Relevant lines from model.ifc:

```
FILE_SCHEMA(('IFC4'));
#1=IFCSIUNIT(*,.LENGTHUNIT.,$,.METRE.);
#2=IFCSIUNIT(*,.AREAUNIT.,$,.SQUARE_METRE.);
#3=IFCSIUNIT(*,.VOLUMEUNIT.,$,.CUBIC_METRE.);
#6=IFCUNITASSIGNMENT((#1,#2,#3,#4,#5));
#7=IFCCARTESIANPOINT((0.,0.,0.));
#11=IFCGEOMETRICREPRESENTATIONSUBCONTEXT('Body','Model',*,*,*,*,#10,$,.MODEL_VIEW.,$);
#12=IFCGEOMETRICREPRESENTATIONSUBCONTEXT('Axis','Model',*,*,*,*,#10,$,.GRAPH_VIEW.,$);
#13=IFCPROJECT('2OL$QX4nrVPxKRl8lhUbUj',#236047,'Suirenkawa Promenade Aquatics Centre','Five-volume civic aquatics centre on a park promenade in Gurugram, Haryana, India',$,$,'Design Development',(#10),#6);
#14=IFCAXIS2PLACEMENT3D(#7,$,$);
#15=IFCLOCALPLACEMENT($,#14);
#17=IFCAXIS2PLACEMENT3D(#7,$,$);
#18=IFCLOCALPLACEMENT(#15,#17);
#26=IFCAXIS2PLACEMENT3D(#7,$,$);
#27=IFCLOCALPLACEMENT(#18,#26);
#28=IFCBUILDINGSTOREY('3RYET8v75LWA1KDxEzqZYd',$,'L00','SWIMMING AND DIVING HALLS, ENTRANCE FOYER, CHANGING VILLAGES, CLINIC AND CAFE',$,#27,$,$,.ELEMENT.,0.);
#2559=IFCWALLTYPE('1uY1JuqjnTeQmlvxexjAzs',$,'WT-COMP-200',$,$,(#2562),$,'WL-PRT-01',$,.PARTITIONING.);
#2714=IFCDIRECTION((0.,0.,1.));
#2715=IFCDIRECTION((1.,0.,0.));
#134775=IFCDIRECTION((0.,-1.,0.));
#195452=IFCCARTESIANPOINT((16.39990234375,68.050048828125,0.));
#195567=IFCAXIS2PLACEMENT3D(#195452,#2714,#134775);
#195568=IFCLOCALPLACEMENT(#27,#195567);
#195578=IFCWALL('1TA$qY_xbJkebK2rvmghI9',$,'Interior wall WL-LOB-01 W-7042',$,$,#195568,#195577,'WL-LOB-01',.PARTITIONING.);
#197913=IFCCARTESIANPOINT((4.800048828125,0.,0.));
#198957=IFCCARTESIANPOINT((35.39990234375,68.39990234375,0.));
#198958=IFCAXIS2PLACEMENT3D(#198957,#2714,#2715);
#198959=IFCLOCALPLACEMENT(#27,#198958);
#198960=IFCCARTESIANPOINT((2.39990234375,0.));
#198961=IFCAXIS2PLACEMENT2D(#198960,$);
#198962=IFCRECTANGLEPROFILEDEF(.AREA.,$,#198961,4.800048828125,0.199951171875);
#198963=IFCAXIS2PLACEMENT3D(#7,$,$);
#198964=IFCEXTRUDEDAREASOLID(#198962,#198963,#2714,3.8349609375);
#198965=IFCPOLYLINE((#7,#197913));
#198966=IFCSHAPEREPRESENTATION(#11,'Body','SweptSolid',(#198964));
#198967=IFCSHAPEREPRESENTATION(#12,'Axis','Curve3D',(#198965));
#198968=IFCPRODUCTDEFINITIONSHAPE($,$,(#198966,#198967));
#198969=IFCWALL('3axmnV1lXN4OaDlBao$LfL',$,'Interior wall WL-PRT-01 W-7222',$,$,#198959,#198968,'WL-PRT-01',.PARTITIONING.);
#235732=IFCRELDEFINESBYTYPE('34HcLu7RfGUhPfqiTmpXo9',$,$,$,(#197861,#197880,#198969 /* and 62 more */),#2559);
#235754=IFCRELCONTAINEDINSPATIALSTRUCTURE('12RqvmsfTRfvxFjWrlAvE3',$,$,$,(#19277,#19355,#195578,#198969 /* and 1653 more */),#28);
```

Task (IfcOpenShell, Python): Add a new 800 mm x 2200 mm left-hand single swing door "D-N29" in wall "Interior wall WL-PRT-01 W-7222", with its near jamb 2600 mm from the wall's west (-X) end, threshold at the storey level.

```python
import numpy as np
import ifcopenshell
import ifcopenshell.api.feature
import ifcopenshell.api.geometry
import ifcopenshell.api.root
import ifcopenshell.api.spatial
import ifcopenshell.geom
import ifcopenshell.util.element
import ifcopenshell.util.placement
import ifcopenshell.util.representation
import ifcopenshell.util.shape
import ifcopenshell.util.unit

model = ifcopenshell.open("model.ifc")
unit_scale = ifcopenshell.util.unit.calculate_unit_scale(model)
settings = ifcopenshell.geom.settings()


def volume(element):
    """Net volume in cubic metres, openings subtracted."""
    shape = ifcopenshell.geom.create_shape(settings, element)
    return ifcopenshell.util.shape.get_volume(shape.geometry)


wall = model.by_guid("3axmnV1lXN4OaDlBao$LfL")
storey = ifcopenshell.util.element.get_container(wall, ifc_class="IfcBuildingStorey")
context = ifcopenshell.util.representation.get_context(model, "Model", "Body", "MODEL_VIEW")
before = volume(wall)

width, height, from_end, sill = 0.8, 2.2, 2.6, 0.0  # metres

# The wall runs along its own X axis, and the end named is its -X end.
wall_shape = ifcopenshell.geom.create_shape(settings, wall)
x, y, z = ifcopenshell.util.shape.get_vertices(wall_shape.geometry).T
start = x.min() + from_end
face, thickness = float(y.min()), float(y.max() - y.min())
wall_matrix = ifcopenshell.util.placement.get_local_placement(wall.ObjectPlacement)
level = ifcopenshell.util.placement.get_local_placement(storey.ObjectPlacement)[2, 3]


def in_wall(x, y):
    """Placement at x, y metres in the wall's axes, at sill height."""
    matrix = wall_matrix.copy()
    matrix[:, 3] = wall_matrix @ np.array([x / unit_scale, y / unit_scale, 0.0, 1.0])
    matrix[2, 3] = level + sill / unit_scale
    return matrix


# Opening: a box that overshoots both wall faces by 50 mm.
opening = ifcopenshell.api.root.create_entity(model, ifc_class="IfcOpeningElement", predefined_type="OPENING")
box = ifcopenshell.api.geometry.add_wall_representation(
    model, context=context, length=width, height=height, thickness=thickness + 0.1
)
ifcopenshell.api.geometry.assign_representation(model, product=opening, representation=box)
ifcopenshell.api.geometry.edit_object_placement(model, product=opening, matrix=in_wall(start, face - 0.05), is_si=False)
ifcopenshell.api.feature.add_feature(model, feature=opening, element=wall)

door = ifcopenshell.api.root.create_entity(model, ifc_class="IfcDoor", name="D-N29", predefined_type="DOOR")
door.OverallWidth, door.OverallHeight = width / unit_scale, height / unit_scale
door.OperationType = "SINGLE_SWING_LEFT"
body = ifcopenshell.api.geometry.add_door_representation(
    model,
    context=context,
    overall_width=door.OverallWidth,
    overall_height=door.OverallHeight,
    operation_type="SINGLE_SWING_LEFT",
    lining_properties={"LiningDepth": thickness / unit_scale, "ThresholdDepth": thickness / unit_scale},
)
ifcopenshell.api.geometry.assign_representation(model, product=door, representation=body)
ifcopenshell.api.spatial.assign_container(model, products=[door], relating_structure=storey)
ifcopenshell.api.feature.add_filling(model, opening=opening, element=door)

# The lining spans the wall, so the door starts at the wall face.
ifcopenshell.api.geometry.edit_object_placement(model, product=door, matrix=in_wall(start, face), is_si=False)

after = volume(wall)

print(f"wall volume {before:.3f} -> {after:.3f} m3")

model.write("model-out.ifc")
```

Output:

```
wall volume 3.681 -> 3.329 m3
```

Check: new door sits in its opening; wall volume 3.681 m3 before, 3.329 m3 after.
